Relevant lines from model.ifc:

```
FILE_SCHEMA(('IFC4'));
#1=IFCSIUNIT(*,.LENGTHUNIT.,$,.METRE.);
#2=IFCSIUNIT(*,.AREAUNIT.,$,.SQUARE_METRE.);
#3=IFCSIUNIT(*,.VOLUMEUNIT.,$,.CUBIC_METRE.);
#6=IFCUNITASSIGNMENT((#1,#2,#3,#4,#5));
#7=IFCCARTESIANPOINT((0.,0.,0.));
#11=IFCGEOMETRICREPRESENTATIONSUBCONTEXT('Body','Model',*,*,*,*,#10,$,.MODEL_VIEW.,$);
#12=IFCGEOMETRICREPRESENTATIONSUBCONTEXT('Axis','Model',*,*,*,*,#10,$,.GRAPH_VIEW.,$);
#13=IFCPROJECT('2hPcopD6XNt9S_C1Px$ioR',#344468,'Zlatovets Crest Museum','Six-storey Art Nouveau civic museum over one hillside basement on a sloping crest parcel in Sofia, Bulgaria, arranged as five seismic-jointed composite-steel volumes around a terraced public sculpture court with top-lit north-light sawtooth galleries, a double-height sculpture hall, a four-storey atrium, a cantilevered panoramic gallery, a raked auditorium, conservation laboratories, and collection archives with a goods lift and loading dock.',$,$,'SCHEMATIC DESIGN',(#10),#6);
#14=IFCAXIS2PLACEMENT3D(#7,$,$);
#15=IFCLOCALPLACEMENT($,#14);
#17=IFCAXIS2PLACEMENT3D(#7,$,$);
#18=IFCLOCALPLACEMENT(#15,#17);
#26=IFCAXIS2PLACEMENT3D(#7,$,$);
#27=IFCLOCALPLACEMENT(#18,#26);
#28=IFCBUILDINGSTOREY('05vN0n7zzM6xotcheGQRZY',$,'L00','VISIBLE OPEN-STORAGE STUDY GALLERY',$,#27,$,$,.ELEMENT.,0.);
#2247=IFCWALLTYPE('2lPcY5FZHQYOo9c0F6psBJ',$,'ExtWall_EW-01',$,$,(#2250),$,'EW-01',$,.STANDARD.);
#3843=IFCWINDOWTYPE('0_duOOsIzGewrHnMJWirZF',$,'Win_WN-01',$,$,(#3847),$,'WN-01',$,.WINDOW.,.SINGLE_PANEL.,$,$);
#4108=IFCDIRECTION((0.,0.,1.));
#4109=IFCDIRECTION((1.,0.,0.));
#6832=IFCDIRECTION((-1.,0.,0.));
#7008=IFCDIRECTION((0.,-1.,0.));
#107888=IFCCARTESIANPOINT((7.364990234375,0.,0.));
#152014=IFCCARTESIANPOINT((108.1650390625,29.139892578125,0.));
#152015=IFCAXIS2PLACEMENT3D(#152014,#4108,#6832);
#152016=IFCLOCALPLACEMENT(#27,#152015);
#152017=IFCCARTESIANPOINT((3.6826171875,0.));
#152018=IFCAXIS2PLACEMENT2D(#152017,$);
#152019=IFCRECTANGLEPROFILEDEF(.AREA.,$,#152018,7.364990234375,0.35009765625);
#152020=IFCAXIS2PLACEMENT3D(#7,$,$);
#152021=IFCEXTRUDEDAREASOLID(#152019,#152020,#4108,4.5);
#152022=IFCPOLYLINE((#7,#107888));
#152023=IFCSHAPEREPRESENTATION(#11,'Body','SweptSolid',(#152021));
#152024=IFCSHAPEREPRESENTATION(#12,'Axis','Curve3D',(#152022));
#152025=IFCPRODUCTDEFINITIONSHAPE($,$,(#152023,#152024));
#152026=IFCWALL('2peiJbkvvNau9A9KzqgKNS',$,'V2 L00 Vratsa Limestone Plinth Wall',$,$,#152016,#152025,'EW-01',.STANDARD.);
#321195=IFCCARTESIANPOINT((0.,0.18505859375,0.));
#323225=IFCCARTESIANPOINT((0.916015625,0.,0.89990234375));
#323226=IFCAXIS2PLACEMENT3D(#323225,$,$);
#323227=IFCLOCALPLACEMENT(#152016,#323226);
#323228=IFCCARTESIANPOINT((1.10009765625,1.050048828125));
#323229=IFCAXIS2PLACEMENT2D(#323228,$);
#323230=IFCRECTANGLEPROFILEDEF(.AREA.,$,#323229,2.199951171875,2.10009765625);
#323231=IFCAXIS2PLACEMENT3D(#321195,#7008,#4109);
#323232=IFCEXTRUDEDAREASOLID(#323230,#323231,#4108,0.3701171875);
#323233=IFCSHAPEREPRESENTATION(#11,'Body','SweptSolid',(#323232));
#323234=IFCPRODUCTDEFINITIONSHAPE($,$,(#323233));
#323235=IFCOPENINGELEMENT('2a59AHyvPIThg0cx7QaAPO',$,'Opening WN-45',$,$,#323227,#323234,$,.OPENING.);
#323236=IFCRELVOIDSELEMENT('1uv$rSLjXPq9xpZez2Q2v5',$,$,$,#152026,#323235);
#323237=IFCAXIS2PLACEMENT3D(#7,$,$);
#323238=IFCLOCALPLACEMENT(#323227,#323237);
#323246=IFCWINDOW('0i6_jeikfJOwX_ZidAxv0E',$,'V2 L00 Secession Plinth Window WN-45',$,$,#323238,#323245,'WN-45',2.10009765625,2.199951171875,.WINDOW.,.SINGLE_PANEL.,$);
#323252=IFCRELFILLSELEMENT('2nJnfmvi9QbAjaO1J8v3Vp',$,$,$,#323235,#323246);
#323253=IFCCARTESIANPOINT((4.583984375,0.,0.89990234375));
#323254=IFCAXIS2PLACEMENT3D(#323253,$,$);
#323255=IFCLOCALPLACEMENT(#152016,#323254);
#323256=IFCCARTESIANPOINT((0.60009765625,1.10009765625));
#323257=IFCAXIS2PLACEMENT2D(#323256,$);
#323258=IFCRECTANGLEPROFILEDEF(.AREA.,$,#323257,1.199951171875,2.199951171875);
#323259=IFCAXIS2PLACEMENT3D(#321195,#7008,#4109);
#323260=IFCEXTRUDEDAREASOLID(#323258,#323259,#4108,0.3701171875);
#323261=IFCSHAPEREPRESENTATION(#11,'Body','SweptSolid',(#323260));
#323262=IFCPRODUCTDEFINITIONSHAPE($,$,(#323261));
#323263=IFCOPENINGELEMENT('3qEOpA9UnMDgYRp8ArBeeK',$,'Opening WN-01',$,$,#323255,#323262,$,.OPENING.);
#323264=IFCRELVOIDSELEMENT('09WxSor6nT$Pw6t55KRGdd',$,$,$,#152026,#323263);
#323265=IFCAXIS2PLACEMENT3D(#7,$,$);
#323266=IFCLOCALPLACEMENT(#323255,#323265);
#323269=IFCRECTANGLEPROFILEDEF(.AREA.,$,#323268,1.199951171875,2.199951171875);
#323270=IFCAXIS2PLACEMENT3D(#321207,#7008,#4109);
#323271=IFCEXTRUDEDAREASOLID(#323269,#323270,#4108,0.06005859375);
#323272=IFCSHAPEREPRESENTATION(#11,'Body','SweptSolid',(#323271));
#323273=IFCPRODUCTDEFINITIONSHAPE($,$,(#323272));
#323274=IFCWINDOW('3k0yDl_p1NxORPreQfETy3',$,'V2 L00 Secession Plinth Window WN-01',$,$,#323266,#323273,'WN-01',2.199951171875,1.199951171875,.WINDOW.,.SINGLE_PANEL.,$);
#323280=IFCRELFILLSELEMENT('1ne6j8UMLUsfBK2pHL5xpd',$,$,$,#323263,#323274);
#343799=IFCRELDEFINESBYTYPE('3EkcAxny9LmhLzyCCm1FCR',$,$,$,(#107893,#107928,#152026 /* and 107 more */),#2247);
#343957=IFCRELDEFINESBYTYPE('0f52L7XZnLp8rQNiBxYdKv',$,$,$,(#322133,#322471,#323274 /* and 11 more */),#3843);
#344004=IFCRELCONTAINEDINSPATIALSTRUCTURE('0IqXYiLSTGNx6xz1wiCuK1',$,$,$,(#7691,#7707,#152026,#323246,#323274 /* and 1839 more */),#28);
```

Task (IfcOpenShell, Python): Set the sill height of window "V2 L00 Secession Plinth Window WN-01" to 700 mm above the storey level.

```python
import numpy as np
import ifcopenshell
import ifcopenshell.api.geometry
import ifcopenshell.geom
import ifcopenshell.util.element
import ifcopenshell.util.placement
import ifcopenshell.util.shape
import ifcopenshell.util.unit

model = ifcopenshell.open("model.ifc")
unit_scale = ifcopenshell.util.unit.calculate_unit_scale(model)

window = model.by_guid("3k0yDl_p1NxORPreQfETy3")
opening = window.FillsVoids[0].RelatingOpeningElement
storey = ifcopenshell.util.element.get_container(window, ifc_class="IfcBuildingStorey")
level = ifcopenshell.util.placement.get_local_placement(storey.ObjectPlacement)[2, 3]

# The opening's origin need not be at the sill, so measure its lowest point.
shape = ifcopenshell.geom.create_shape(ifcopenshell.geom.settings(), opening)
bottom = ifcopenshell.util.shape.get_shape_bottom_elevation(shape, shape.geometry) / unit_scale
dz = level + 0.7 / unit_scale - bottom

shift = np.array([0.0, 0.0, dz])
# The window is placed relative to its opening, so it follows when the opening moves.
matrix = ifcopenshell.util.placement.get_local_placement(opening.ObjectPlacement)
matrix[:3, 3] += shift
ifcopenshell.api.geometry.edit_object_placement(
    model, product=opening, matrix=matrix, is_si=False, should_transform_children=True
)

print(f"moved by {dz * unit_scale:+.3f} m")

model.write("model_rev.ifc")
```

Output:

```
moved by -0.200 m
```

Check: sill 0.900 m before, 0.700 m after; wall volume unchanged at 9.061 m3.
